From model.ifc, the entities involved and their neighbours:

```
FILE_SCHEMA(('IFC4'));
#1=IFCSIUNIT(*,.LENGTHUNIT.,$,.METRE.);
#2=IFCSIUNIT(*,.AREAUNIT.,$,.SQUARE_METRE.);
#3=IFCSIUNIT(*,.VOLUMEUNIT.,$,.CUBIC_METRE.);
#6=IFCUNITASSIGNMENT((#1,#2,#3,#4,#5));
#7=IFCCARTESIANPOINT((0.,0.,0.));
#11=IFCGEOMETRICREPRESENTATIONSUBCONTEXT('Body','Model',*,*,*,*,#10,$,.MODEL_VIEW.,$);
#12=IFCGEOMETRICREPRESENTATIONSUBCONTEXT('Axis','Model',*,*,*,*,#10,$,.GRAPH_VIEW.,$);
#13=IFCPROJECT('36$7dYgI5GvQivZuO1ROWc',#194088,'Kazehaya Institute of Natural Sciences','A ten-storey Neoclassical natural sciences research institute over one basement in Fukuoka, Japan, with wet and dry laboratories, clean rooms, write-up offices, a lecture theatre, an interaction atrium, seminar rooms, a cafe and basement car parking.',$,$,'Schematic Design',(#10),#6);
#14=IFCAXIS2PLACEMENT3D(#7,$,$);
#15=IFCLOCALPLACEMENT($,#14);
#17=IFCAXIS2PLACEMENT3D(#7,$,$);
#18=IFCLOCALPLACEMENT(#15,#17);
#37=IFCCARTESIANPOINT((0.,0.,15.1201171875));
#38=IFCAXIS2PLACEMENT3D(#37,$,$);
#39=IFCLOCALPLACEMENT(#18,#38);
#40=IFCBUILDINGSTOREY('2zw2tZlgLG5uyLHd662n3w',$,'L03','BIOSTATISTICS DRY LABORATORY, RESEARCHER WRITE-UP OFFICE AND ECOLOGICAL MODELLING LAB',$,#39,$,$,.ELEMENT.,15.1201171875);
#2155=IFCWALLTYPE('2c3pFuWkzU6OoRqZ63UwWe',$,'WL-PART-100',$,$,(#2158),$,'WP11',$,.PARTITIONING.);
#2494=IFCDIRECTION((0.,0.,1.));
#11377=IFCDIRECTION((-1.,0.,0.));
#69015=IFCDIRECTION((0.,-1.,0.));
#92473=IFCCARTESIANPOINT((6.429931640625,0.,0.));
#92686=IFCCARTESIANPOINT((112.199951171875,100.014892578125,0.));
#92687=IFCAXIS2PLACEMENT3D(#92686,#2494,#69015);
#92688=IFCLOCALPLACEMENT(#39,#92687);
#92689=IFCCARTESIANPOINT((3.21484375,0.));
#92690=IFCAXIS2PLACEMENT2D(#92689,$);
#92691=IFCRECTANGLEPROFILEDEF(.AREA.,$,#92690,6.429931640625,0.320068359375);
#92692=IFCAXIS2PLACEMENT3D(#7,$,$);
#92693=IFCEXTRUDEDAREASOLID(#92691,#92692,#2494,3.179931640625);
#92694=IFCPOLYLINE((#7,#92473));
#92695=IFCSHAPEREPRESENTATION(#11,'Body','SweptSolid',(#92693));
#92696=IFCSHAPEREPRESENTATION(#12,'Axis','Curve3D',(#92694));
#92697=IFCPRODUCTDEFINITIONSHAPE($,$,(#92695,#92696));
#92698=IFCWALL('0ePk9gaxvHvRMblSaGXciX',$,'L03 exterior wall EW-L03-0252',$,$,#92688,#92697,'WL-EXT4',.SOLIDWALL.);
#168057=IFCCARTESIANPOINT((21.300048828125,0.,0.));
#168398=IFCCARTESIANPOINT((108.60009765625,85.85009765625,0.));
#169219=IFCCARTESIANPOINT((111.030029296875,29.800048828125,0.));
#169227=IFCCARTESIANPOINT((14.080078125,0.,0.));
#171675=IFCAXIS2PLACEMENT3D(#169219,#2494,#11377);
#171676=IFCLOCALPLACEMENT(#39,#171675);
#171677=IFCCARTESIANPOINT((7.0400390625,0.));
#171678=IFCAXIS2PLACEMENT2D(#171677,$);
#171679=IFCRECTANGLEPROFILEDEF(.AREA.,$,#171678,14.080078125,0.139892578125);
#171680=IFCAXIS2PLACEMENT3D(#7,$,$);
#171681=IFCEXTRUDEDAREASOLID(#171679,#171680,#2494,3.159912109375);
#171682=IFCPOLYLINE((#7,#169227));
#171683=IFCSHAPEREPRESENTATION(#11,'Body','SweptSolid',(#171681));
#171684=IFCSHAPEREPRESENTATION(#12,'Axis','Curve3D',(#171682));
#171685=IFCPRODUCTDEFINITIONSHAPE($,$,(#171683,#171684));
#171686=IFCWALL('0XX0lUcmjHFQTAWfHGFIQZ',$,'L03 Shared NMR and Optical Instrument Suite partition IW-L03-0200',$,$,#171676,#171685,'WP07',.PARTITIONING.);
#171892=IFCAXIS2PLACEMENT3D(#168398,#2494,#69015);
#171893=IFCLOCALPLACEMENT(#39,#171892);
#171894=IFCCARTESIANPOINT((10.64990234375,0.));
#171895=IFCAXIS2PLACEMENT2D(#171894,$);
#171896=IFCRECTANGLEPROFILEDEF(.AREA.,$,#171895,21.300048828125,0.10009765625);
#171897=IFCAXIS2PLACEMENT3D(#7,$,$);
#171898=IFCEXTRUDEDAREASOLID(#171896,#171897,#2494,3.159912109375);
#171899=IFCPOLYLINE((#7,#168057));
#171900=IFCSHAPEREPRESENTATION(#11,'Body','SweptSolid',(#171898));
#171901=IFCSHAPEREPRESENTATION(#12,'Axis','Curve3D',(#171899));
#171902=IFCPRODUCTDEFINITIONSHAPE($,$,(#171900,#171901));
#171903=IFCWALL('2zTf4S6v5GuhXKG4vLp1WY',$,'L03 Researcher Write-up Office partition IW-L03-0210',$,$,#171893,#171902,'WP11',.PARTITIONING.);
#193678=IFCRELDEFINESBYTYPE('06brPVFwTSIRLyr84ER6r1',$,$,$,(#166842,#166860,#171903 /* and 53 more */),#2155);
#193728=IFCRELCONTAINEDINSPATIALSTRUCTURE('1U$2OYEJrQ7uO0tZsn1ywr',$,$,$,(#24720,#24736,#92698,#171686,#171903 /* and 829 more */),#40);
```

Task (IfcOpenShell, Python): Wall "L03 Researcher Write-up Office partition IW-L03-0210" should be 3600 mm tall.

```python
import ifcopenshell
import ifcopenshell.geom
import ifcopenshell.util.representation
import ifcopenshell.util.shape
import ifcopenshell.util.unit

model = ifcopenshell.open("model.ifc")
unit_scale = ifcopenshell.util.unit.calculate_unit_scale(model)
settings = ifcopenshell.geom.settings()


def volume(element):
    """Net volume in cubic metres, openings subtracted."""
    shape = ifcopenshell.geom.create_shape(settings, element)
    return ifcopenshell.util.shape.get_volume(shape.geometry)


wall = model.by_guid("2zTf4S6v5GuhXKG4vLp1WY")
before = volume(wall)

body = ifcopenshell.util.representation.get_representation(wall, "Model", "Body")
solid = body.Items[0]
old_height = solid.Depth
solid.Depth = 3.6 / unit_scale
after = volume(wall)

print(f"height {old_height:g} -> {solid.Depth:g}, volume {before:.3f} -> {after:.3f} m3")

model.write("model-out.ifc")
```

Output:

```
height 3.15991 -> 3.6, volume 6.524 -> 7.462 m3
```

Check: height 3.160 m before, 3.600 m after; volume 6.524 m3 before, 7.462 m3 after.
